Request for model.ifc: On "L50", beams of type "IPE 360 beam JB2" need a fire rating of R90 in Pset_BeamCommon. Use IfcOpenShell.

First a look at what the model holds.

```python
import ifcopenshell
import ifcopenshell.util.element

model = ifcopenshell.open("model.ifc")
print(model.schema)
storey = next(s for s in model.by_type("IfcBuildingStorey") if s.Name == "L50")
beams = [e for e in ifcopenshell.util.element.get_decomposition(storey) if e.is_a("IfcBeam")]
seen = {}
for e in beams:
    element_type = ifcopenshell.util.element.get_type(e)
    key = (element_type.Name if element_type != e and element_type else None, ifcopenshell.util.element.get_pset(e, "Pset_BeamCommon", "FireRating"))
    seen[key] = seen.get(key, 0) + 1
for (name, value), count in sorted(seen.items(), key=str):
    print(count, "x", name, "|", value)
```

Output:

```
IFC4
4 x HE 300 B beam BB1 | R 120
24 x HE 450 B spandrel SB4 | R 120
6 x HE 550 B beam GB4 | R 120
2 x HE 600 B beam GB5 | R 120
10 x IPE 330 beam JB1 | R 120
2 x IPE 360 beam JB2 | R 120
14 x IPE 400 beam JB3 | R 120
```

```python
import ifcopenshell
import ifcopenshell.api.pset
import ifcopenshell.util.element

model = ifcopenshell.open("model.ifc")

storey = next(s for s in model.by_type("IfcBuildingStorey") if s.Name == "L50")
beams = [e for e in ifcopenshell.util.element.get_decomposition(storey) if e.is_a("IfcBeam")]

count = 0
for e in beams:
    element_type = ifcopenshell.util.element.get_type(e)
    if element_type in (None, e) or element_type.Name != "IPE 360 beam JB2":
        continue
    found = ifcopenshell.util.element.get_pset(e, "Pset_BeamCommon", should_inherit=False)
    if found:
        pset = model.by_id(found["id"])
        if len(ifcopenshell.util.element.get_elements_by_pset(pset)) > 1:
            pset = ifcopenshell.api.pset.unshare_pset(model, products=[e], pset=pset)[0]
    else:
        pset = ifcopenshell.api.pset.add_pset(model, product=e, name="Pset_BeamCommon")
    ifcopenshell.api.pset.edit_pset(model, pset=pset, properties={"FireRating": "R90"})
    count += 1

print(count, "beams updated")

model.write("model_v2.ifc")
```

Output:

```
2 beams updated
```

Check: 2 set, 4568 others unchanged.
